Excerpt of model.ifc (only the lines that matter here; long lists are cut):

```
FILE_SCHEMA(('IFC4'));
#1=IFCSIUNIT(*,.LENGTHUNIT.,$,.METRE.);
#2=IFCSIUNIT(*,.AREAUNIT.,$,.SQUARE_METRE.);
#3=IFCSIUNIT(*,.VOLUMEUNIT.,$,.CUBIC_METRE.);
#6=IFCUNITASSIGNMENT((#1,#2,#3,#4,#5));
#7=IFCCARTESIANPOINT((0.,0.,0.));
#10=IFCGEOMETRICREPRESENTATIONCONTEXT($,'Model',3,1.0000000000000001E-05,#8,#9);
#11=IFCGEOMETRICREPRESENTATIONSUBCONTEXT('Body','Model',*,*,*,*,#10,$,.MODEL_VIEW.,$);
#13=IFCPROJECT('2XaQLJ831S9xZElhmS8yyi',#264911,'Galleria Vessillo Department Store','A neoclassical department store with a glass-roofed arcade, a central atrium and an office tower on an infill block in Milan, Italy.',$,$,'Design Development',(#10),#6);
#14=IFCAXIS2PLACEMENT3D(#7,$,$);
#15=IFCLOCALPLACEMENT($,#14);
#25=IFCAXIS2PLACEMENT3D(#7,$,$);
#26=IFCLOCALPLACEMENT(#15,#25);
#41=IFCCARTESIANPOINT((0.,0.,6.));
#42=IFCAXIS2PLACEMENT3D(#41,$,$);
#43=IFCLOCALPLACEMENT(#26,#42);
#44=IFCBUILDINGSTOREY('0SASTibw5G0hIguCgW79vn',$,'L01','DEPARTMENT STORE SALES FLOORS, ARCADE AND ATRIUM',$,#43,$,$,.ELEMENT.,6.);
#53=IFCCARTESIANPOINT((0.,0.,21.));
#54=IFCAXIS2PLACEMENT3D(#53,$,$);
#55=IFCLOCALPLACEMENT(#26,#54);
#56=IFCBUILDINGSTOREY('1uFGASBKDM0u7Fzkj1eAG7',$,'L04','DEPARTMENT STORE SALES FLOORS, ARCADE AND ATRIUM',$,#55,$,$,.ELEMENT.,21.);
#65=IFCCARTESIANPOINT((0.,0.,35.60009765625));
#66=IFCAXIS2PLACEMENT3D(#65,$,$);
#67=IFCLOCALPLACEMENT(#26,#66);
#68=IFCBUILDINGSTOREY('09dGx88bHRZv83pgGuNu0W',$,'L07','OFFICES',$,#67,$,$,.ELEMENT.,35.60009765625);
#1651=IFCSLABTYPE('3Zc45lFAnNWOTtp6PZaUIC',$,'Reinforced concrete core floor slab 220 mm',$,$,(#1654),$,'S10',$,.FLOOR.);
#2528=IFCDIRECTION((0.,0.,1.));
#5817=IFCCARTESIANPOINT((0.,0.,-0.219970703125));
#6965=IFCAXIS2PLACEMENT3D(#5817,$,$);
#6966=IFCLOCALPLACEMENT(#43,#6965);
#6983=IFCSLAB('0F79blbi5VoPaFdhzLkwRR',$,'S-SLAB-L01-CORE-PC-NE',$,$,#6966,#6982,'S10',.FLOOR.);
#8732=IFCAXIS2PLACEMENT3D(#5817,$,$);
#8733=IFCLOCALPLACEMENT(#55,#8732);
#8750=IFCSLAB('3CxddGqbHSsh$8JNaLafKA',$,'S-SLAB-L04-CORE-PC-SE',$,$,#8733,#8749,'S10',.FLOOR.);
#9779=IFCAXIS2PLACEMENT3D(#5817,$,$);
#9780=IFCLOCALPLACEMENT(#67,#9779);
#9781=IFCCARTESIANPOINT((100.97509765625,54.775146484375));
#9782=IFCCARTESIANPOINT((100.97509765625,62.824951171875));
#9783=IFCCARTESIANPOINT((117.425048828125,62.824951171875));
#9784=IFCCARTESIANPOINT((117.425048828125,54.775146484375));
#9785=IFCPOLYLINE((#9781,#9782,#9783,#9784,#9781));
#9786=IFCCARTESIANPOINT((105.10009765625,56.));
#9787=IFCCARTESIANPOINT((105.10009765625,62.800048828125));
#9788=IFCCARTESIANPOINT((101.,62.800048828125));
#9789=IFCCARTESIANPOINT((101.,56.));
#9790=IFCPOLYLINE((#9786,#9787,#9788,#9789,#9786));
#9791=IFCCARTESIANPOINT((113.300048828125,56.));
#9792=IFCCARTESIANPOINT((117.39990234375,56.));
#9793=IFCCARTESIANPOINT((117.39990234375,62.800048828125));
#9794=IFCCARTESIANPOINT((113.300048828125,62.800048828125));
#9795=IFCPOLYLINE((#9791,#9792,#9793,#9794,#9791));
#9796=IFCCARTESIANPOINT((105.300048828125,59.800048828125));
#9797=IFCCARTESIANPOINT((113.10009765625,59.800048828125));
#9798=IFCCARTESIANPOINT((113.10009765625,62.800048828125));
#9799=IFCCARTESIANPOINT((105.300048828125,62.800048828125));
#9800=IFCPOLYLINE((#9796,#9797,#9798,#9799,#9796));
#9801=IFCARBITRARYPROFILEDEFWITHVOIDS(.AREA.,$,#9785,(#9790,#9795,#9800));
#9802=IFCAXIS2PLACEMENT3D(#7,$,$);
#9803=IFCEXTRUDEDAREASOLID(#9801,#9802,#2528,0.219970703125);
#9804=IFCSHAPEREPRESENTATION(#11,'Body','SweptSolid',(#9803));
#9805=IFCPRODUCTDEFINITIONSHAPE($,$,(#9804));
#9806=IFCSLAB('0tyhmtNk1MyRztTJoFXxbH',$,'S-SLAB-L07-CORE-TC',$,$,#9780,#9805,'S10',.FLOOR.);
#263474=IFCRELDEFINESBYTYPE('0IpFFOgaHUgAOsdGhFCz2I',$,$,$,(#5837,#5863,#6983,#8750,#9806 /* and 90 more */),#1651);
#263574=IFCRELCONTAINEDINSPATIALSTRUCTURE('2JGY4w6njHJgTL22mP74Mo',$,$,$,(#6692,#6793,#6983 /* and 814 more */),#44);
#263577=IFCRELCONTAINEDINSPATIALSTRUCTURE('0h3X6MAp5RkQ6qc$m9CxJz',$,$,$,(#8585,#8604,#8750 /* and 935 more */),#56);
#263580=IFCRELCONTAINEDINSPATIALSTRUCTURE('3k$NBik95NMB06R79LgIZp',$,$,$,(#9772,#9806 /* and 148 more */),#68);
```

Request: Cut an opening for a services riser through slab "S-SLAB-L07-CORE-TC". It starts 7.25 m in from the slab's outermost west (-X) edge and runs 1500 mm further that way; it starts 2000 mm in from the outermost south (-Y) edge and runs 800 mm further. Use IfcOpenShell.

```python
import numpy as np
import ifcopenshell
import ifcopenshell.api.feature
import ifcopenshell.api.geometry
import ifcopenshell.api.root
import ifcopenshell.geom
import ifcopenshell.util.placement
import ifcopenshell.util.representation
import ifcopenshell.util.shape
import ifcopenshell.util.unit

model = ifcopenshell.open("model.ifc")
unit_scale = ifcopenshell.util.unit.calculate_unit_scale(model)
settings = ifcopenshell.geom.settings()


def volume(element):
    """Net volume in cubic metres, openings subtracted."""
    shape = ifcopenshell.geom.create_shape(settings, element)
    return ifcopenshell.util.shape.get_volume(shape.geometry)


slab = model.by_guid("0tyhmtNk1MyRztTJoFXxbH")
before = volume(slab)

# Extent in the slab's own axes, in metres. The edges named are its -X and -Y sides.
slab_shape = ifcopenshell.geom.create_shape(settings, slab)
vertices = ifcopenshell.util.shape.get_vertices(slab_shape.geometry)
x_min, y_min, bottom = vertices.min(axis=0)
top = vertices[:, 2].max()

opening = ifcopenshell.api.root.create_entity(model, ifc_class="IfcOpeningElement", name="Services riser opening", predefined_type="OPENING")
context = ifcopenshell.util.representation.get_context(model, "Model", "Body", "MODEL_VIEW")
width, depth = 1.5, 0.8
outline = [(0.0, 0.0), (width, 0.0), (width, depth), (0.0, depth), (0.0, 0.0)]
# Overshoot both faces by 50 mm so the cut is clean.
shape = ifcopenshell.api.geometry.add_slab_representation(
    model, context=context, depth=top - bottom + 0.1, polyline=outline
)
ifcopenshell.api.geometry.assign_representation(model, product=opening, representation=shape)

matrix = ifcopenshell.util.placement.get_local_placement(slab.ObjectPlacement)
matrix[:, 3] = matrix @ np.append(np.array([x_min + 7.25, y_min + 2, bottom - 0.05]) / unit_scale, 1.0)
ifcopenshell.api.geometry.edit_object_placement(model, product=opening, matrix=matrix, is_si=False)
ifcopenshell.api.feature.add_feature(model, feature=opening, element=slab)

after = volume(slab)

print(f"slab volume {before:.3f} -> {after:.3f} m3")

model.write("model_updated.ifc")
```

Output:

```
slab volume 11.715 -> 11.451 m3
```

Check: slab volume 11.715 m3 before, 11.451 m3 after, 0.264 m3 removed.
